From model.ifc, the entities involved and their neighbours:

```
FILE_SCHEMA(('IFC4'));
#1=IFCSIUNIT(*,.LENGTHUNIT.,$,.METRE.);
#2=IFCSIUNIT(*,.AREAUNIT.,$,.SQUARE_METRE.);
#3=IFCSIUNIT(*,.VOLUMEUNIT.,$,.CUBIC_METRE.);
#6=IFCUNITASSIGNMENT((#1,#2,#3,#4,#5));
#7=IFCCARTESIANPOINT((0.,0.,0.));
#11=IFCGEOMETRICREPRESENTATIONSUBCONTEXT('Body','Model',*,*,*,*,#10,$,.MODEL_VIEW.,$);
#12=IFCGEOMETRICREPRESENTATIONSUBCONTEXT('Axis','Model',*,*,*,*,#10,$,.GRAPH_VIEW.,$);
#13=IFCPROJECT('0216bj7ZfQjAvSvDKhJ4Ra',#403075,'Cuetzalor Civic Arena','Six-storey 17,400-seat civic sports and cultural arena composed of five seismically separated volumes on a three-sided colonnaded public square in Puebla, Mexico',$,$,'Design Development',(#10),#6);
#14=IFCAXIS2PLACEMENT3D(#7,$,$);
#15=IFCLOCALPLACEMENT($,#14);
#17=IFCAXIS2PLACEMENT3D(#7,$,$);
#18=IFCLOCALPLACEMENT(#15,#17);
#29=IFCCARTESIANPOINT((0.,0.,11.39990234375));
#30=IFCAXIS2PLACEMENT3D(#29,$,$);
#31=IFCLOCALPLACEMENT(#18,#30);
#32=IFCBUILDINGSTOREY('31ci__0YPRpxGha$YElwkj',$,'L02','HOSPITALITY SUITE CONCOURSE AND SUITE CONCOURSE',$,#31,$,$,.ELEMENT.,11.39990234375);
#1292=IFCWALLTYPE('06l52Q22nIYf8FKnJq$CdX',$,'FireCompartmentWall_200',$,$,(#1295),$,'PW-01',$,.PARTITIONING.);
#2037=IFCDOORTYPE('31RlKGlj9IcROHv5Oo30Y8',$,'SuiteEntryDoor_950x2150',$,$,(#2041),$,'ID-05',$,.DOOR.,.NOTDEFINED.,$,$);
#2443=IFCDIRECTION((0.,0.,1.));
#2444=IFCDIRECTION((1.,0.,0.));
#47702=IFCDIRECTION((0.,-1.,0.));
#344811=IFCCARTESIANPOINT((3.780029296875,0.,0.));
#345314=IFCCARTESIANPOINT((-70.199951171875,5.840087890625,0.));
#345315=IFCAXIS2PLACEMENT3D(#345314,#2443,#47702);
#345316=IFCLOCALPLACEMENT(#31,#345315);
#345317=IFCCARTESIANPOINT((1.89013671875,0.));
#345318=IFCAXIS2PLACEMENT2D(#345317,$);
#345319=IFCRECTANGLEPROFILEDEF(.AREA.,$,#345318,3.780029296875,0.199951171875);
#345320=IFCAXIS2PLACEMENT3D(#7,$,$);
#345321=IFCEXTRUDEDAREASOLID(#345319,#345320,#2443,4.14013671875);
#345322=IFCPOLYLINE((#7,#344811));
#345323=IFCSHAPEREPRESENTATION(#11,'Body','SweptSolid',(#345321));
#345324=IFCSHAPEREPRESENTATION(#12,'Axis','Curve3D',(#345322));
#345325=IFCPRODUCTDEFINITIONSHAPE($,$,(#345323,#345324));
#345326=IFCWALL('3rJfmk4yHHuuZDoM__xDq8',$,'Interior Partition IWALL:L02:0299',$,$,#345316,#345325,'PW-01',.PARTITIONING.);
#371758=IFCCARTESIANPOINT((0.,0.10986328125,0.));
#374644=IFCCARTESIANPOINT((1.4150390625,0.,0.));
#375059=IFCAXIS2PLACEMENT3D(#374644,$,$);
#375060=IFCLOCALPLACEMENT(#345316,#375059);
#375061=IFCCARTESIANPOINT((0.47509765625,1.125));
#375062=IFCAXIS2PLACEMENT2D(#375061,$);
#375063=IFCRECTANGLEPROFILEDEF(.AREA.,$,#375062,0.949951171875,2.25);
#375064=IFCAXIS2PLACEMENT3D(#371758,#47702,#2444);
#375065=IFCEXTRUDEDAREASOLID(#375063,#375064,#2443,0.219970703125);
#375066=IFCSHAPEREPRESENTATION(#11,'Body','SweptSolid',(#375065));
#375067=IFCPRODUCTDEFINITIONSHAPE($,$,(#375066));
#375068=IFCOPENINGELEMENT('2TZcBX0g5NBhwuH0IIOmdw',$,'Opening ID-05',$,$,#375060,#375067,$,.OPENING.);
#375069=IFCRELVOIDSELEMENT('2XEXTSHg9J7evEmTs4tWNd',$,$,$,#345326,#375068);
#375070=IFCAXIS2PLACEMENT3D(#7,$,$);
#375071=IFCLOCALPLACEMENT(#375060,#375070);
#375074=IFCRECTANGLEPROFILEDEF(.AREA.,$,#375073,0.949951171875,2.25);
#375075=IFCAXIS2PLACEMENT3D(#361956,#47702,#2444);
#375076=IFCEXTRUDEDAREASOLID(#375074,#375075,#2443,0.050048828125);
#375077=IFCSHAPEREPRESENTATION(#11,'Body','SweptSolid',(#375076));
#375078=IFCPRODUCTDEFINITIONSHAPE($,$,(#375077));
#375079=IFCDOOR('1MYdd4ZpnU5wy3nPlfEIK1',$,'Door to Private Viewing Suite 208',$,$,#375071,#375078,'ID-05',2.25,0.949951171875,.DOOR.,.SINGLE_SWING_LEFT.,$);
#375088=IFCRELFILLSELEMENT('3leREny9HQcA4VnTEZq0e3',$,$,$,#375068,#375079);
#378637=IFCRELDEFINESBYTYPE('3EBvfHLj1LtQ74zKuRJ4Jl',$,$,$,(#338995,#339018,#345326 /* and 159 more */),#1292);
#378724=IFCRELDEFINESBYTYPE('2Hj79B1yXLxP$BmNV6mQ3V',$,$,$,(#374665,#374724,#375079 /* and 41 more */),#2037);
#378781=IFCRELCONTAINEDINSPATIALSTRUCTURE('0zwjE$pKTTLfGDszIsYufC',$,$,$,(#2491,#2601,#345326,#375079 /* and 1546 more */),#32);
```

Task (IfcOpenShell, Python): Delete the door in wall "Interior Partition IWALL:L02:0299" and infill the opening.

```python
import ifcopenshell
import ifcopenshell.api.feature
import ifcopenshell.api.root
import ifcopenshell.geom
import ifcopenshell.util.shape

model = ifcopenshell.open("model.ifc")
settings = ifcopenshell.geom.settings()


def volume(element):
    """Net volume in cubic metres, openings subtracted."""
    shape = ifcopenshell.geom.create_shape(settings, element)
    return ifcopenshell.util.shape.get_volume(shape.geometry)


door = model.by_guid("1MYdd4ZpnU5wy3nPlfEIK1")
opening = door.FillsVoids[0].RelatingOpeningElement
wall = opening.VoidsElements[0].RelatingBuildingElement
before = volume(wall)

ifcopenshell.api.root.remove_product(model, product=door)
ifcopenshell.api.feature.remove_feature(model, feature=opening)

after = volume(wall)

print(f"wall volume {before:.3f} -> {after:.3f} m3")

model.write("model_rev.ifc")
```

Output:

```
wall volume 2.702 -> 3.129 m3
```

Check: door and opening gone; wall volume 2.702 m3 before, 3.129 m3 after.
